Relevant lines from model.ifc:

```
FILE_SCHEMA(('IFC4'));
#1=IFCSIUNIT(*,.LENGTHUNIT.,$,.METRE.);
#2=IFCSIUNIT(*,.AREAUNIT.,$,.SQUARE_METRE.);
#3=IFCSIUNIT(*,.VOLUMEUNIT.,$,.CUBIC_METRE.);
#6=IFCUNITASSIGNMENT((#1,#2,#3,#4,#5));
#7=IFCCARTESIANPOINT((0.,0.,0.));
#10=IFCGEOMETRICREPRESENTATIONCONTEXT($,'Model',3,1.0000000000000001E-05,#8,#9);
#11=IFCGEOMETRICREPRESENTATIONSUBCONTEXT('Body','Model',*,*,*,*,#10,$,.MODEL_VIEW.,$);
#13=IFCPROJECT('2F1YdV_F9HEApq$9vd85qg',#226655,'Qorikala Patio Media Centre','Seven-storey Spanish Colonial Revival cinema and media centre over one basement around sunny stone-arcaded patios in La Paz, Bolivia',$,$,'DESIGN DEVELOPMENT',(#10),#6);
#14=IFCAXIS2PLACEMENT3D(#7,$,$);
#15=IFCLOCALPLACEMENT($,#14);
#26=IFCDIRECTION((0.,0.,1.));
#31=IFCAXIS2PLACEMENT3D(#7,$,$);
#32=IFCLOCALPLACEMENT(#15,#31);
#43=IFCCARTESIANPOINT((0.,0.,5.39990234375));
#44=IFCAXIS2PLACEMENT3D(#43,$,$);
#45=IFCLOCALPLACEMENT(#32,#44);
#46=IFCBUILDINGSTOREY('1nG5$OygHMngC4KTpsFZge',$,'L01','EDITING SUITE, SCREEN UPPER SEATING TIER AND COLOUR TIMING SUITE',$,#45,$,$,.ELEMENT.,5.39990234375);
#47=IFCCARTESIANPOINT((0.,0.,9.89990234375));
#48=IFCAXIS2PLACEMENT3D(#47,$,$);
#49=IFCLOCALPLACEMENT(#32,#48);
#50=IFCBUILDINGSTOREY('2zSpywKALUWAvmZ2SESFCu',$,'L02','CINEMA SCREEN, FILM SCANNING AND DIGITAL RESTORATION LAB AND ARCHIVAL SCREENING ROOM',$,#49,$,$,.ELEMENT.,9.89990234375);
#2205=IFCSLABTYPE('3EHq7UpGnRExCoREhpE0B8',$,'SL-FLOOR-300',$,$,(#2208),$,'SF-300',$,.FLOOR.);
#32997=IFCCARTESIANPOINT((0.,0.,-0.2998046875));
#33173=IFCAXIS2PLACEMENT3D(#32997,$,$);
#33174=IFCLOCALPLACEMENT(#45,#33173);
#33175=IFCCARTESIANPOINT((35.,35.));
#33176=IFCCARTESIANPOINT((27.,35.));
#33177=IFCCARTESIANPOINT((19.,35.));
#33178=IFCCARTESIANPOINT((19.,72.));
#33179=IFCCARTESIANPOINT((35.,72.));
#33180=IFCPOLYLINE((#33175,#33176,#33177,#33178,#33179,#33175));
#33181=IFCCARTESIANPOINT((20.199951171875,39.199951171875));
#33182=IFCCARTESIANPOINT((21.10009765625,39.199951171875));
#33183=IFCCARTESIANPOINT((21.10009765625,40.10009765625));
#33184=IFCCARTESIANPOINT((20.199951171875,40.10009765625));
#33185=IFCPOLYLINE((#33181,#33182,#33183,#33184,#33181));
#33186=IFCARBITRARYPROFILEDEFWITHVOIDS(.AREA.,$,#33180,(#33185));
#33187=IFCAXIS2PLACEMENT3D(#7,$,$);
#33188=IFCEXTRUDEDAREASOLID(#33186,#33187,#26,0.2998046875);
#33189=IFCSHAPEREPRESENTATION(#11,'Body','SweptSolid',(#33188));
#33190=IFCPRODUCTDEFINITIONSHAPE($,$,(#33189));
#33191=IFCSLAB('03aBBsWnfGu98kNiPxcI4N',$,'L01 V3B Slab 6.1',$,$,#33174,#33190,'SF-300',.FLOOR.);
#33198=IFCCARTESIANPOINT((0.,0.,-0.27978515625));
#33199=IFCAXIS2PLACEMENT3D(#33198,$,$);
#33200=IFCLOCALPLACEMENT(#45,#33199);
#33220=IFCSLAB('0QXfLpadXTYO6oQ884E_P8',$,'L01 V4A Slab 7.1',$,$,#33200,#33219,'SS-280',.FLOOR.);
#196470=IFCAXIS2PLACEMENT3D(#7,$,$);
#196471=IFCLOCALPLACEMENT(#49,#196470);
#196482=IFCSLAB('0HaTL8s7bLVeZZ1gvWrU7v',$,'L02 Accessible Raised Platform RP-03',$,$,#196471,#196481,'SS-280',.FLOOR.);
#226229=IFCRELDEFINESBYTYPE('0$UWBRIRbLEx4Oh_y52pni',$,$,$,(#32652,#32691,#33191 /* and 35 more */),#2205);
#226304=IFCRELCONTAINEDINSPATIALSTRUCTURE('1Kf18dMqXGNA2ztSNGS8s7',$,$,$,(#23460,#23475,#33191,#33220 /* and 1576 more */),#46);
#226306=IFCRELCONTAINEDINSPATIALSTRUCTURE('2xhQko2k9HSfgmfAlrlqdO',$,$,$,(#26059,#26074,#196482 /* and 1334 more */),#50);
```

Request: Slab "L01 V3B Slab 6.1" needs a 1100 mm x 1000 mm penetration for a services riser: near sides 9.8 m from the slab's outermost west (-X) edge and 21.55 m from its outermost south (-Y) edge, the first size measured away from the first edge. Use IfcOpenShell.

```python
import numpy as np
import ifcopenshell
import ifcopenshell.api.feature
import ifcopenshell.api.geometry
import ifcopenshell.api.root
import ifcopenshell.geom
import ifcopenshell.util.placement
import ifcopenshell.util.representation
import ifcopenshell.util.shape
import ifcopenshell.util.unit

model = ifcopenshell.open("model.ifc")
unit_scale = ifcopenshell.util.unit.calculate_unit_scale(model)
settings = ifcopenshell.geom.settings()


def volume(element):
    """Net volume in cubic metres, openings subtracted."""
    shape = ifcopenshell.geom.create_shape(settings, element)
    return ifcopenshell.util.shape.get_volume(shape.geometry)


slab = model.by_id(33191)
before = volume(slab)

# Extent in the slab's own axes, in metres. The edges named are its -X and -Y sides.
slab_shape = ifcopenshell.geom.create_shape(settings, slab)
vertices = ifcopenshell.util.shape.get_vertices(slab_shape.geometry)
x_min, y_min, bottom = vertices.min(axis=0)
top = vertices[:, 2].max()

opening = ifcopenshell.api.root.create_entity(model, ifc_class="IfcOpeningElement", name="Services riser opening", predefined_type="OPENING")
context = ifcopenshell.util.representation.get_context(model, "Model", "Body", "MODEL_VIEW")
width, depth = 1.1, 1
outline = [(0.0, 0.0), (width, 0.0), (width, depth), (0.0, depth), (0.0, 0.0)]
# Overshoot both faces by 50 mm so the cut is clean.
shape = ifcopenshell.api.geometry.add_slab_representation(
    model, context=context, depth=top - bottom + 0.1, polyline=outline
)
ifcopenshell.api.geometry.assign_representation(model, product=opening, representation=shape)

matrix = ifcopenshell.util.placement.get_local_placement(slab.ObjectPlacement)
matrix[:, 3] = matrix @ np.append(np.array([x_min + 9.8, y_min + 21.55, bottom - 0.05]) / unit_scale, 1.0)
ifcopenshell.api.geometry.edit_object_placement(model, product=opening, matrix=matrix, is_si=False)
ifcopenshell.api.feature.add_feature(model, feature=opening, element=slab)

after = volume(slab)

print(f"slab volume {before:.3f} -> {after:.3f} m3")

model.write("model_rev.ifc")
```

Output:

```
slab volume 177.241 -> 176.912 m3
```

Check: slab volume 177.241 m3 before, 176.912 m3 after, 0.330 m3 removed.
